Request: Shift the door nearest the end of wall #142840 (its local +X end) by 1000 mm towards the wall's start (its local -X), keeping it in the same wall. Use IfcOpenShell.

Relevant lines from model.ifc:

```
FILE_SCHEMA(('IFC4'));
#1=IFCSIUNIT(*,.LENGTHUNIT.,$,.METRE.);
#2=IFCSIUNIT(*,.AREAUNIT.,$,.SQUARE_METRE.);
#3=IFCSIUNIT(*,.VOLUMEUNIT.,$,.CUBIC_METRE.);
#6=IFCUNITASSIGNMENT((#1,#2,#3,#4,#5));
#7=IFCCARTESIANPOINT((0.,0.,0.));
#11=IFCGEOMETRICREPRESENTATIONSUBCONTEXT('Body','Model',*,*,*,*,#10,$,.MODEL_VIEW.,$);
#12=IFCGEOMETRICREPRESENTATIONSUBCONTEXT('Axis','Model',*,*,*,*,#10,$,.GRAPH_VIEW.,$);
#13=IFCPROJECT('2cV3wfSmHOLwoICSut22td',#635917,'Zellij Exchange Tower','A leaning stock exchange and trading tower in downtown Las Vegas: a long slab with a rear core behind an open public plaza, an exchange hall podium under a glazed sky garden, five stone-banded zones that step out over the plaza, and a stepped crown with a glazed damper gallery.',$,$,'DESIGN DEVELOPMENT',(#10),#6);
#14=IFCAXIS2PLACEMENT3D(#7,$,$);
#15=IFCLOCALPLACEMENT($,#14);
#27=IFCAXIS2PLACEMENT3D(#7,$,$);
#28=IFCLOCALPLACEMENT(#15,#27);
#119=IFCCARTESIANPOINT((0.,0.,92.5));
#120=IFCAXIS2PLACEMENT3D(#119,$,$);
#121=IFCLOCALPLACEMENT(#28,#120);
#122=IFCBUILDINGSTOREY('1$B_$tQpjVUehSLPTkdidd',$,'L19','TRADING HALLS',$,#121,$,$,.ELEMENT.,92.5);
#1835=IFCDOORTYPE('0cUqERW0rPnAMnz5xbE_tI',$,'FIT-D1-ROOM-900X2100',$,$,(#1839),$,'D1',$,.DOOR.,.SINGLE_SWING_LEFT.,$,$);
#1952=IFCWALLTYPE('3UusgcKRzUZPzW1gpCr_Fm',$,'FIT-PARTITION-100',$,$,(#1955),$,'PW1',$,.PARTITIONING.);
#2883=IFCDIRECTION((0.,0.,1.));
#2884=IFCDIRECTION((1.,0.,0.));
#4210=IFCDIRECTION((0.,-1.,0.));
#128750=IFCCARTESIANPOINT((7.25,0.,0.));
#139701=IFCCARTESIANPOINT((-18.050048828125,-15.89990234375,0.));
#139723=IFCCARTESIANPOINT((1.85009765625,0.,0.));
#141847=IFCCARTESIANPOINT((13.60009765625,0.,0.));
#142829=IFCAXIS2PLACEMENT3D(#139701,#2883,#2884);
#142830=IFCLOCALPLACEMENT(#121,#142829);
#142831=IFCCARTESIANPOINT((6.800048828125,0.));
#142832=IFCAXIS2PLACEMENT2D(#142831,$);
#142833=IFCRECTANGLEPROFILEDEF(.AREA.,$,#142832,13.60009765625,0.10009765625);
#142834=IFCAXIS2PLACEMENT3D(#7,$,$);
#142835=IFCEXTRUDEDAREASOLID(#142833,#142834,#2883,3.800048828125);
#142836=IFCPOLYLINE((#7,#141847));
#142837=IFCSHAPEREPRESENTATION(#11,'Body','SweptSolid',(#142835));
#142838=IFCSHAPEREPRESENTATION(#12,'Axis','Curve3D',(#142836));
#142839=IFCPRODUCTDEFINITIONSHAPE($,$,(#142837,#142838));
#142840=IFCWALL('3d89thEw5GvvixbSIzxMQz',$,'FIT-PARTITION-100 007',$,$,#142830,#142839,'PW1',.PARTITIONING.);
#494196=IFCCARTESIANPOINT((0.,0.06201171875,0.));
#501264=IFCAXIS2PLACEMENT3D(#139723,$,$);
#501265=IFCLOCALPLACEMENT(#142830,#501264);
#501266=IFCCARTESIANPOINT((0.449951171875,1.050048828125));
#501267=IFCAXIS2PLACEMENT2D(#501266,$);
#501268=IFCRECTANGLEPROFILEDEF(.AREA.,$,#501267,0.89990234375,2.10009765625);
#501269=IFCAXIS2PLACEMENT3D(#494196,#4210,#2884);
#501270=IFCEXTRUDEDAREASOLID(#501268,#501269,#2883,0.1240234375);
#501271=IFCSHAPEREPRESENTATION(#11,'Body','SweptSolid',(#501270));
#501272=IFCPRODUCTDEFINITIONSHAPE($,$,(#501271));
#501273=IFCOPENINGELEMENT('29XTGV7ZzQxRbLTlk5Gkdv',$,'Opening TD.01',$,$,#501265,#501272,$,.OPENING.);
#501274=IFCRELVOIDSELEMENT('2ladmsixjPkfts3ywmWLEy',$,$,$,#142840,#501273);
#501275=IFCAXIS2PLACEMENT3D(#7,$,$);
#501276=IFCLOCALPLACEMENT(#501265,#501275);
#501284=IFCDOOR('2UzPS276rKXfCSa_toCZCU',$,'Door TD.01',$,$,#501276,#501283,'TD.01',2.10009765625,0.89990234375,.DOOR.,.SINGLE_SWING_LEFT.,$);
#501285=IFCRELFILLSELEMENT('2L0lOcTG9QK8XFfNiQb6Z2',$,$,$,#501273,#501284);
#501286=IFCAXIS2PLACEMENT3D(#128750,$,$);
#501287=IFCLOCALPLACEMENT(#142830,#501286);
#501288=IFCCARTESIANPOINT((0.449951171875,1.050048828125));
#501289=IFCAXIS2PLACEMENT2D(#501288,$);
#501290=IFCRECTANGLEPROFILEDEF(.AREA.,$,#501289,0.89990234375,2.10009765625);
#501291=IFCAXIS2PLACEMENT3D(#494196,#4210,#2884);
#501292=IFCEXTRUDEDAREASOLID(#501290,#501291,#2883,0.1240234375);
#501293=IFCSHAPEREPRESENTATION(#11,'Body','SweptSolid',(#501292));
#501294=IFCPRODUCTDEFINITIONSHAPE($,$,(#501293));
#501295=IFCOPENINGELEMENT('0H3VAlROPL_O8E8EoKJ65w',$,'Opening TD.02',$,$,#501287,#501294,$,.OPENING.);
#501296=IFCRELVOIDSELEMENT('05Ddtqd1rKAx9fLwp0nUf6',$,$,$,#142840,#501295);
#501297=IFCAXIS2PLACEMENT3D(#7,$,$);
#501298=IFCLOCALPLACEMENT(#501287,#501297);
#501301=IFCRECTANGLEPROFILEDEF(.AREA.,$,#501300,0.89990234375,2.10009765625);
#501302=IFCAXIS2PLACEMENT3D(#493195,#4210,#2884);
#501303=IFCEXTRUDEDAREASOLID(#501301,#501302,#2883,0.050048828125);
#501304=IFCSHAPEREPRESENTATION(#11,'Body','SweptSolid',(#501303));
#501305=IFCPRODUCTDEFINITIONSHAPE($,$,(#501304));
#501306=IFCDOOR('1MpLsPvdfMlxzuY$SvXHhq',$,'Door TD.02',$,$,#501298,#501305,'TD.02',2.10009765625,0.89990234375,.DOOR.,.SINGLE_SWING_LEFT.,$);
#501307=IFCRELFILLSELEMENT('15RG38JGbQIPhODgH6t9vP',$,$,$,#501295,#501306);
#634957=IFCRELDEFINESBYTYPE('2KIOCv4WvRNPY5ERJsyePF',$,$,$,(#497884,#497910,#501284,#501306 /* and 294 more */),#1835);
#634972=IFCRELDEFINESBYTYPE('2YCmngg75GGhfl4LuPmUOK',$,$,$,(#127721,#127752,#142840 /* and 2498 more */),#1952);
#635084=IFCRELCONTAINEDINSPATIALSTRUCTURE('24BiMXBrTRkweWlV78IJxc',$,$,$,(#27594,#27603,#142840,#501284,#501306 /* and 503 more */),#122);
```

```python
import ifcopenshell
import ifcopenshell.api.geometry
import ifcopenshell.util.placement

model = ifcopenshell.open("model.ifc")

door = model.by_id(501306)
opening = door.FillsVoids[0].RelatingOpeningElement
wall = opening.VoidsElements[0].RelatingBuildingElement

wall_matrix = ifcopenshell.util.placement.get_local_placement(wall.ObjectPlacement)
shift = wall_matrix[:3, 0] * -1.0
before = ifcopenshell.util.placement.get_local_placement(door.ObjectPlacement)[:3, 3].copy()

# The door is placed relative to its opening, so it follows when the opening moves.
matrix = ifcopenshell.util.placement.get_local_placement(opening.ObjectPlacement)
matrix[:3, 3] += shift
ifcopenshell.api.geometry.edit_object_placement(
    model, product=opening, matrix=matrix, is_si=False, should_transform_children=True
)

after = ifcopenshell.util.placement.get_local_placement(door.ObjectPlacement)[:3, 3]
print("door moved by", (after - before).round(3) + 0.0)

model.write("model_updated.ifc")
```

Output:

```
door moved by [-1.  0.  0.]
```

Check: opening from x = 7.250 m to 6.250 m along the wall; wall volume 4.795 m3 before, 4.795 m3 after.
